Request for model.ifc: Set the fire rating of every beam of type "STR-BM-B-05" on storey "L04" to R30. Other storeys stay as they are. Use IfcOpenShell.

First a look at what the model holds.

```python
import ifcopenshell
import ifcopenshell.util.element

model = ifcopenshell.open("model.ifc")
print(model.schema)
storey = next(s for s in model.by_type("IfcBuildingStorey") if s.Name == "L04")
beams = [e for e in ifcopenshell.util.element.get_decomposition(storey) if e.is_a("IfcBeam")]
seen = {}
for e in beams:
    element_type = ifcopenshell.util.element.get_type(e)
    key = (element_type.Name if element_type != e and element_type else None, ifcopenshell.util.element.get_pset(e, "Pset_BeamCommon", "FireRating"))
    seen[key] = seen.get(key, 0) + 1
for (name, value), count in sorted(seen.items(), key=str):
    print(count, "x", name, "|", value)
```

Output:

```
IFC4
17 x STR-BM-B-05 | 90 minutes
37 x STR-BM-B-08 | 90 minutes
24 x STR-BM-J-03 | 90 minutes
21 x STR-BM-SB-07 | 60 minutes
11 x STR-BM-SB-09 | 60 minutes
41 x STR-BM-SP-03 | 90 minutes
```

```python
import ifcopenshell
import ifcopenshell.api.pset
import ifcopenshell.util.element

model = ifcopenshell.open("model.ifc")

storey = next(s for s in model.by_type("IfcBuildingStorey") if s.Name == "L04")
beams = [e for e in ifcopenshell.util.element.get_decomposition(storey) if e.is_a("IfcBeam")]

count = 0
for e in beams:
    element_type = ifcopenshell.util.element.get_type(e)
    if element_type in (None, e) or element_type.Name != "STR-BM-B-05":
        continue
    # add_pset returns the element's existing set when there is one.
    pset = ifcopenshell.api.pset.add_pset(model, product=e, name="Pset_BeamCommon")
    ifcopenshell.api.pset.edit_pset(model, pset=pset, properties={"FireRating": "R30"})
    count += 1

print(count, "beams updated")

model.write("model_edited.ifc")
```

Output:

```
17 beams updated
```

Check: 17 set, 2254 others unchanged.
